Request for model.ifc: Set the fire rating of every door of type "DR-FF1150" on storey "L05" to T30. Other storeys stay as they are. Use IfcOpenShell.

First a look at what the model holds.

```python
import ifcopenshell
import ifcopenshell.util.element

model = ifcopenshell.open("model.ifc")
print(model.schema)
storey = next(s for s in model.by_type("IfcBuildingStorey") if s.Name == "L05")
doors = [e for e in ifcopenshell.util.element.get_decomposition(storey) if e.is_a("IfcDoor")]
seen = {}
for e in doors:
    element_type = ifcopenshell.util.element.get_type(e)
    key = (element_type.Name if element_type != e and element_type else None, ifcopenshell.util.element.get_pset(e, "Pset_DoorCommon", "FireRating"))
    seen[key] = seen.get(key, 0) + 1
for (name, value), count in sorted(seen.items(), key=str):
    print(count, "x", name, "|", value)
```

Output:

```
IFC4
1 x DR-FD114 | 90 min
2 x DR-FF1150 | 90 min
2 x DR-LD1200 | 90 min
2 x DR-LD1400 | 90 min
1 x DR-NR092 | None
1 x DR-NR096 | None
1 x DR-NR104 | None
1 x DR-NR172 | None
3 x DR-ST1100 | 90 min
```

```python
import ifcopenshell
import ifcopenshell.api.pset
import ifcopenshell.util.element

model = ifcopenshell.open("model.ifc")

storey = next(s for s in model.by_type("IfcBuildingStorey") if s.Name == "L05")
doors = [e for e in ifcopenshell.util.element.get_decomposition(storey) if e.is_a("IfcDoor")]

count = 0
for e in doors:
    element_type = ifcopenshell.util.element.get_type(e)
    if element_type in (None, e) or element_type.Name != "DR-FF1150":
        continue
    # add_pset returns the element's existing set when there is one.
    pset = ifcopenshell.api.pset.add_pset(model, product=e, name="Pset_DoorCommon")
    ifcopenshell.api.pset.edit_pset(model, pset=pset, properties={"FireRating": "T30"})
    count += 1

print(count, "doors updated")

model.write("model_edited.ifc")
```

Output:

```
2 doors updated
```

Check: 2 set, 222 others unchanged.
